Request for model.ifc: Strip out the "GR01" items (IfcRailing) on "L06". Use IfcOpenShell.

First a look at what the model holds.

```python
import ifcopenshell
import ifcopenshell.util.element

model = ifcopenshell.open("model.ifc")
print(model.schema)
storey = next(s for s in model.by_type("IfcBuildingStorey") if s.Name == "L06")
railings = [e for e in ifcopenshell.util.element.get_decomposition(storey) if e.is_a("IfcRailing")]
seen = {}
for e in railings:
    element_type = ifcopenshell.util.element.get_type(e)
    name = element_type.Name if element_type not in (None, e) else None
    seen[name] = seen.get(name, 0) + 1
for name, count in sorted(seen.items(), key=str):
    print(count, "x", name)
```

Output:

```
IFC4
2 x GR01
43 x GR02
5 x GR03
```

```python
import ifcopenshell
import ifcopenshell.api.root
import ifcopenshell.util.element

model = ifcopenshell.open("model.ifc")

storey = next(s for s in model.by_type("IfcBuildingStorey") if s.Name == "L06")
railings = [e for e in ifcopenshell.util.element.get_decomposition(storey) if e.is_a("IfcRailing")]
targets = [e for e in railings if (t := ifcopenshell.util.element.get_type(e)) not in (None, e) and t.Name == "GR01"]

for e in targets:
    ifcopenshell.api.root.remove_product(model, product=e)
print(len(targets), "removed")

model.write("model_rev.ifc")
```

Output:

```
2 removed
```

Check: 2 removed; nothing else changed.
